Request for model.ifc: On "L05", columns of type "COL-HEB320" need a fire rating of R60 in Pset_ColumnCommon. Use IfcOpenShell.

First a look at what the model holds.

```python
import ifcopenshell
import ifcopenshell.util.element

model = ifcopenshell.open("model.ifc")
print(model.schema)
storey = next(s for s in model.by_type("IfcBuildingStorey") if s.Name == "L05")
columns = [e for e in ifcopenshell.util.element.get_decomposition(storey) if e.is_a("IfcColumn")]
seen = {}
for e in columns:
    element_type = ifcopenshell.util.element.get_type(e)
    key = (element_type.Name if element_type != e and element_type else None, ifcopenshell.util.element.get_pset(e, "Pset_ColumnCommon", "FireRating"))
    seen[key] = seen.get(key, 0) + 1
for (name, value), count in sorted(seen.items(), key=str):
    print(count, "x", name, "|", value)
```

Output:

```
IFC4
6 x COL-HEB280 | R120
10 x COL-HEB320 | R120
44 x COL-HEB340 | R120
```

```python
import ifcopenshell
import ifcopenshell.api.pset
import ifcopenshell.util.element

model = ifcopenshell.open("model.ifc")

storey = next(s for s in model.by_type("IfcBuildingStorey") if s.Name == "L05")
columns = [e for e in ifcopenshell.util.element.get_decomposition(storey) if e.is_a("IfcColumn")]

count = 0
for e in columns:
    element_type = ifcopenshell.util.element.get_type(e)
    if element_type in (None, e) or element_type.Name != "COL-HEB320":
        continue
    # add_pset returns the element's existing set when there is one.
    pset = ifcopenshell.api.pset.add_pset(model, product=e, name="Pset_ColumnCommon")
    ifcopenshell.api.pset.edit_pset(model, pset=pset, properties={"FireRating": "R60"})
    count += 1

print(count, "columns updated")

model.write("model_edited.ifc")
```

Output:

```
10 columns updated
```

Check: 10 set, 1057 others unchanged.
